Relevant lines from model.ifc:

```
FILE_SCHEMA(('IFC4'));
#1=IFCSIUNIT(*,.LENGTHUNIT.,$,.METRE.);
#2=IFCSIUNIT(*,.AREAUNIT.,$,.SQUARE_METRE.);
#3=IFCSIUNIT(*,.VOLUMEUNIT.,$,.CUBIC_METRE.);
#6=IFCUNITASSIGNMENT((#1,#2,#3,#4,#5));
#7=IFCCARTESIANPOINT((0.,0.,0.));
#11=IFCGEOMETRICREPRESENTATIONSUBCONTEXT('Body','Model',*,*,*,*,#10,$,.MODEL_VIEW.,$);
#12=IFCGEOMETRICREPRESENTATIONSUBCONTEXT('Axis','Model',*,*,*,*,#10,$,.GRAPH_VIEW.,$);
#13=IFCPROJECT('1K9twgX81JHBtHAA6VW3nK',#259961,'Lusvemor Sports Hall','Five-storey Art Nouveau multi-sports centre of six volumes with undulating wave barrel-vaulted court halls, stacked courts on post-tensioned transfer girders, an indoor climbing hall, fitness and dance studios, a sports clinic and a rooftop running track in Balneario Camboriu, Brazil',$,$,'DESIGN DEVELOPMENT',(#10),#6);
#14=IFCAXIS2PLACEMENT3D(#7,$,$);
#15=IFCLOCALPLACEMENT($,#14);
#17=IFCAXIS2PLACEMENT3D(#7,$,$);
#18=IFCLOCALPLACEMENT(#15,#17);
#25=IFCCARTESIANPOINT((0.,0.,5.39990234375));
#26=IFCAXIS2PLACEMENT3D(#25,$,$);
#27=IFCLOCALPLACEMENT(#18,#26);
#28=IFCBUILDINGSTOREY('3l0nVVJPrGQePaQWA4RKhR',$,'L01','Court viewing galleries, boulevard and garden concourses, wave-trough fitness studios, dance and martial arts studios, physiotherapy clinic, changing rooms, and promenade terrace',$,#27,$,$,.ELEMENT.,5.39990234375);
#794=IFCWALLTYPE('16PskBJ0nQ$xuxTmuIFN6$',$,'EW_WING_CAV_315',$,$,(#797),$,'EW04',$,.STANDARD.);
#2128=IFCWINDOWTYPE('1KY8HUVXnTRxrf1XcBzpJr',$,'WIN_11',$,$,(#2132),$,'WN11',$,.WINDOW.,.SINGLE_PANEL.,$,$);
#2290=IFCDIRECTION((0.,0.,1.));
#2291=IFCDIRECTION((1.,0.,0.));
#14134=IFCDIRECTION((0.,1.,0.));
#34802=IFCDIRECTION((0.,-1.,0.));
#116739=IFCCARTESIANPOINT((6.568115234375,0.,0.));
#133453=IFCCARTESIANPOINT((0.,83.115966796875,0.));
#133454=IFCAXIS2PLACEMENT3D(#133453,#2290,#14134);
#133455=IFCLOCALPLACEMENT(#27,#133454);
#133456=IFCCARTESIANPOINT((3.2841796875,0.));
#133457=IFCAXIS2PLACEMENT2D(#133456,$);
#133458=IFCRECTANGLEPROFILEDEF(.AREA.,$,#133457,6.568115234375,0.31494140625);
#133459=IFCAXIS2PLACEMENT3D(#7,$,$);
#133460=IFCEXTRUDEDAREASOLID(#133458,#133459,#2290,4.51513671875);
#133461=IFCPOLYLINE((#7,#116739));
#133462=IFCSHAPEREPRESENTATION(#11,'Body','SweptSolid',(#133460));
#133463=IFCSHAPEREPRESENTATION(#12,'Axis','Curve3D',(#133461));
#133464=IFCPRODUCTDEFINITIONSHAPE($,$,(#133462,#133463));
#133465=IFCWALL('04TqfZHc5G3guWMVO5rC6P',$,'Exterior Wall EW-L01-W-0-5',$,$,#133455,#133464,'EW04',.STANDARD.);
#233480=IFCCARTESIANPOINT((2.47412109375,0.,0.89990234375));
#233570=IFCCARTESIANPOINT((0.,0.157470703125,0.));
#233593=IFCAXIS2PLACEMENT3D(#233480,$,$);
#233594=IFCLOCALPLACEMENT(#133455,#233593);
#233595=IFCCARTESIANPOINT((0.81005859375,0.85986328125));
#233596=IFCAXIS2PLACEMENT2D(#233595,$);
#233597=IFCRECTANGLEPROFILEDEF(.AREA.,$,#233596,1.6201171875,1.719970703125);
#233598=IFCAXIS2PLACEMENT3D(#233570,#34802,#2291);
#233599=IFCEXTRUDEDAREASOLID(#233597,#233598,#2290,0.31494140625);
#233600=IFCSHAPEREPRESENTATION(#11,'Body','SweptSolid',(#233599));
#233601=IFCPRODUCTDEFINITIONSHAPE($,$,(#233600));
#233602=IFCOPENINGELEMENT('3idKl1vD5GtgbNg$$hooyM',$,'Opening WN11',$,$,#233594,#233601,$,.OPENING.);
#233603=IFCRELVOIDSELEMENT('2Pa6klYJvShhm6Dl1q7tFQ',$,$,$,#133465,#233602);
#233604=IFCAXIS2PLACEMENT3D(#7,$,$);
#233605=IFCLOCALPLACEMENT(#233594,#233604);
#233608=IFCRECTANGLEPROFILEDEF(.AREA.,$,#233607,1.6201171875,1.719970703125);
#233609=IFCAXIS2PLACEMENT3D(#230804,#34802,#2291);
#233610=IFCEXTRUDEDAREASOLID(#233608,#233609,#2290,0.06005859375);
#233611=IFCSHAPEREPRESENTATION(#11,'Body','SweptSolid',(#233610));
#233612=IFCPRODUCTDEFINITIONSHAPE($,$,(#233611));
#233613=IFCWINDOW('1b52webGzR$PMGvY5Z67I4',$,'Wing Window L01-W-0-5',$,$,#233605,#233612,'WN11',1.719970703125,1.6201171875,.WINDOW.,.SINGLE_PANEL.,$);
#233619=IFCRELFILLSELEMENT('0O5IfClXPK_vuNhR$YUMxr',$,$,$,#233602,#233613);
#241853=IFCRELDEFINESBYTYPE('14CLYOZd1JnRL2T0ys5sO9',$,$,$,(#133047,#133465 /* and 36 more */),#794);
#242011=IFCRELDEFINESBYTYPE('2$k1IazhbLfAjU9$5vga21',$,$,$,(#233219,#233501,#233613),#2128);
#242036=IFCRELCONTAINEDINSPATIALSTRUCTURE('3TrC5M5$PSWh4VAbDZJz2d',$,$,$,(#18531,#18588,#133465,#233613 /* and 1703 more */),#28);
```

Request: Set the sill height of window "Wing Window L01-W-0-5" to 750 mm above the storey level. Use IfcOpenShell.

```python
import numpy as np
import ifcopenshell
import ifcopenshell.api.geometry
import ifcopenshell.geom
import ifcopenshell.util.element
import ifcopenshell.util.placement
import ifcopenshell.util.shape
import ifcopenshell.util.unit

model = ifcopenshell.open("model.ifc")
unit_scale = ifcopenshell.util.unit.calculate_unit_scale(model)

window = model.by_guid("1b52webGzR$PMGvY5Z67I4")
opening = window.FillsVoids[0].RelatingOpeningElement
storey = ifcopenshell.util.element.get_container(window, ifc_class="IfcBuildingStorey")
level = ifcopenshell.util.placement.get_local_placement(storey.ObjectPlacement)[2, 3]

# The opening's origin need not be at the sill, so measure its lowest point.
shape = ifcopenshell.geom.create_shape(ifcopenshell.geom.settings(), opening)
bottom = ifcopenshell.util.shape.get_shape_bottom_elevation(shape, shape.geometry) / unit_scale
dz = level + 0.75 / unit_scale - bottom

shift = np.array([0.0, 0.0, dz])
# The window is placed relative to its opening, so it follows when the opening moves.
matrix = ifcopenshell.util.placement.get_local_placement(opening.ObjectPlacement)
matrix[:3, 3] += shift
ifcopenshell.api.geometry.edit_object_placement(
    model, product=opening, matrix=matrix, is_si=False, should_transform_children=True
)

print(f"moved by {dz * unit_scale:+.3f} m")

model.write("model_rev.ifc")
```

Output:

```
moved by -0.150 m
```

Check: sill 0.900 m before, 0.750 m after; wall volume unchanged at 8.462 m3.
